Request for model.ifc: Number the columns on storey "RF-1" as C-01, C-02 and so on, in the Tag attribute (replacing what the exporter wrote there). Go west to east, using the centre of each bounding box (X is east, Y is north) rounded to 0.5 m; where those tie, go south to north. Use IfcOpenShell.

First a look at what the model holds.

```python
import ifcopenshell
import ifcopenshell.util.element
import ifcopenshell.util.placement

model = ifcopenshell.open("model.ifc")
print(model.schema)
storey = next(s for s in model.by_type("IfcBuildingStorey") if s.Name == "RF-1")
columns = [e for e in ifcopenshell.util.element.get_decomposition(storey) if e.is_a("IfcColumn")]
for e in sorted(columns, key=lambda e: e.id()):
    origin = ifcopenshell.util.placement.get_local_placement(e.ObjectPlacement)[:3, 3]
    print(e.id(), e.Tag, e.Name, origin.round(2) + 0.0, sep=" | ")
```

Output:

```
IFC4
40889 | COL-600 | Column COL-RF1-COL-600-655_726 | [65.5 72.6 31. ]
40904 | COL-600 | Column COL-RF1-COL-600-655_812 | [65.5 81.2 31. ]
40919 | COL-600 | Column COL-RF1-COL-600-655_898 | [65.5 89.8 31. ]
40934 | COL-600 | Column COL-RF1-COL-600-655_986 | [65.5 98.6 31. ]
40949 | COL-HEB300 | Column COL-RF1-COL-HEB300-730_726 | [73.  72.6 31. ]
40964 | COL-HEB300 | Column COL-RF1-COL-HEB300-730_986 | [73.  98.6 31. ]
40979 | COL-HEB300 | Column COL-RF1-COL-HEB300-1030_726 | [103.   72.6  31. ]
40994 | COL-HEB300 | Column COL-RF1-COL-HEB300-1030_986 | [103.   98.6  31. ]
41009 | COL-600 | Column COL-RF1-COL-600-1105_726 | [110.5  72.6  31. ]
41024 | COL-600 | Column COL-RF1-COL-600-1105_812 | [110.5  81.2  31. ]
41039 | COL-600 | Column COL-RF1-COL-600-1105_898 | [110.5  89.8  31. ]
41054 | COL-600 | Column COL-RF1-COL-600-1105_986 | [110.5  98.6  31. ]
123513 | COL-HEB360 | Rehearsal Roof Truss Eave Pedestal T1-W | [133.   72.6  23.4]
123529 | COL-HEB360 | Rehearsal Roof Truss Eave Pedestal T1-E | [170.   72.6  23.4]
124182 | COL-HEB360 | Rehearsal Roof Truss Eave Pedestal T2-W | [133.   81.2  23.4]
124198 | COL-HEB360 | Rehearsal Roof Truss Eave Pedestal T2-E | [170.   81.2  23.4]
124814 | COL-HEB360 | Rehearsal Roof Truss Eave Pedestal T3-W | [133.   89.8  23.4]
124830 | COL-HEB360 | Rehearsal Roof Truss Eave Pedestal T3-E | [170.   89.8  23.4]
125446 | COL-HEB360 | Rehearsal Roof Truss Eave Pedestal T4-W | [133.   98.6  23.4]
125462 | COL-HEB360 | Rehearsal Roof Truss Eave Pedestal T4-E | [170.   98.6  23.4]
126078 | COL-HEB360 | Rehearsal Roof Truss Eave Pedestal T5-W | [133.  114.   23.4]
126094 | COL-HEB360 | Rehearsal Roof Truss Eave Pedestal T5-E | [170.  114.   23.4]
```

```python
import ifcopenshell
import ifcopenshell.geom
import ifcopenshell.util.element
import ifcopenshell.util.shape

model = ifcopenshell.open("model.ifc")
settings = ifcopenshell.geom.settings()
settings.set("use-world-coords", True)


def centre(element):
    shape = ifcopenshell.geom.create_shape(settings, element)
    return ifcopenshell.util.shape.get_bbox_centroid(shape.geometry)


storey = next(s for s in model.by_type("IfcBuildingStorey") if s.Name == "RF-1")
columns = [e for e in ifcopenshell.util.element.get_decomposition(storey) if e.is_a("IfcColumn")]

# Insertion points can sit at a corner or the storey origin, so sort by the geometry (in metres).
centres = {e: centre(e) for e in columns}
columns.sort(key=lambda e: (round(centres[e][0] / 0.5), centres[e][1]))

for i, e in enumerate(columns, start=1):
    number = f"C-{i:02d}"
    e.Tag = number
    print(e.id(), number)

model.write("model-out.ifc")
```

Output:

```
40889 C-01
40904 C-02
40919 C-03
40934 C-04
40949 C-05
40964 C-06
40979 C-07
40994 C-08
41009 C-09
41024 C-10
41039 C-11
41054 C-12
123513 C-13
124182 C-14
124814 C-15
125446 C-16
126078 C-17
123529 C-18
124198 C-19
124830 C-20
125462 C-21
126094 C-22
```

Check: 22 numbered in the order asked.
